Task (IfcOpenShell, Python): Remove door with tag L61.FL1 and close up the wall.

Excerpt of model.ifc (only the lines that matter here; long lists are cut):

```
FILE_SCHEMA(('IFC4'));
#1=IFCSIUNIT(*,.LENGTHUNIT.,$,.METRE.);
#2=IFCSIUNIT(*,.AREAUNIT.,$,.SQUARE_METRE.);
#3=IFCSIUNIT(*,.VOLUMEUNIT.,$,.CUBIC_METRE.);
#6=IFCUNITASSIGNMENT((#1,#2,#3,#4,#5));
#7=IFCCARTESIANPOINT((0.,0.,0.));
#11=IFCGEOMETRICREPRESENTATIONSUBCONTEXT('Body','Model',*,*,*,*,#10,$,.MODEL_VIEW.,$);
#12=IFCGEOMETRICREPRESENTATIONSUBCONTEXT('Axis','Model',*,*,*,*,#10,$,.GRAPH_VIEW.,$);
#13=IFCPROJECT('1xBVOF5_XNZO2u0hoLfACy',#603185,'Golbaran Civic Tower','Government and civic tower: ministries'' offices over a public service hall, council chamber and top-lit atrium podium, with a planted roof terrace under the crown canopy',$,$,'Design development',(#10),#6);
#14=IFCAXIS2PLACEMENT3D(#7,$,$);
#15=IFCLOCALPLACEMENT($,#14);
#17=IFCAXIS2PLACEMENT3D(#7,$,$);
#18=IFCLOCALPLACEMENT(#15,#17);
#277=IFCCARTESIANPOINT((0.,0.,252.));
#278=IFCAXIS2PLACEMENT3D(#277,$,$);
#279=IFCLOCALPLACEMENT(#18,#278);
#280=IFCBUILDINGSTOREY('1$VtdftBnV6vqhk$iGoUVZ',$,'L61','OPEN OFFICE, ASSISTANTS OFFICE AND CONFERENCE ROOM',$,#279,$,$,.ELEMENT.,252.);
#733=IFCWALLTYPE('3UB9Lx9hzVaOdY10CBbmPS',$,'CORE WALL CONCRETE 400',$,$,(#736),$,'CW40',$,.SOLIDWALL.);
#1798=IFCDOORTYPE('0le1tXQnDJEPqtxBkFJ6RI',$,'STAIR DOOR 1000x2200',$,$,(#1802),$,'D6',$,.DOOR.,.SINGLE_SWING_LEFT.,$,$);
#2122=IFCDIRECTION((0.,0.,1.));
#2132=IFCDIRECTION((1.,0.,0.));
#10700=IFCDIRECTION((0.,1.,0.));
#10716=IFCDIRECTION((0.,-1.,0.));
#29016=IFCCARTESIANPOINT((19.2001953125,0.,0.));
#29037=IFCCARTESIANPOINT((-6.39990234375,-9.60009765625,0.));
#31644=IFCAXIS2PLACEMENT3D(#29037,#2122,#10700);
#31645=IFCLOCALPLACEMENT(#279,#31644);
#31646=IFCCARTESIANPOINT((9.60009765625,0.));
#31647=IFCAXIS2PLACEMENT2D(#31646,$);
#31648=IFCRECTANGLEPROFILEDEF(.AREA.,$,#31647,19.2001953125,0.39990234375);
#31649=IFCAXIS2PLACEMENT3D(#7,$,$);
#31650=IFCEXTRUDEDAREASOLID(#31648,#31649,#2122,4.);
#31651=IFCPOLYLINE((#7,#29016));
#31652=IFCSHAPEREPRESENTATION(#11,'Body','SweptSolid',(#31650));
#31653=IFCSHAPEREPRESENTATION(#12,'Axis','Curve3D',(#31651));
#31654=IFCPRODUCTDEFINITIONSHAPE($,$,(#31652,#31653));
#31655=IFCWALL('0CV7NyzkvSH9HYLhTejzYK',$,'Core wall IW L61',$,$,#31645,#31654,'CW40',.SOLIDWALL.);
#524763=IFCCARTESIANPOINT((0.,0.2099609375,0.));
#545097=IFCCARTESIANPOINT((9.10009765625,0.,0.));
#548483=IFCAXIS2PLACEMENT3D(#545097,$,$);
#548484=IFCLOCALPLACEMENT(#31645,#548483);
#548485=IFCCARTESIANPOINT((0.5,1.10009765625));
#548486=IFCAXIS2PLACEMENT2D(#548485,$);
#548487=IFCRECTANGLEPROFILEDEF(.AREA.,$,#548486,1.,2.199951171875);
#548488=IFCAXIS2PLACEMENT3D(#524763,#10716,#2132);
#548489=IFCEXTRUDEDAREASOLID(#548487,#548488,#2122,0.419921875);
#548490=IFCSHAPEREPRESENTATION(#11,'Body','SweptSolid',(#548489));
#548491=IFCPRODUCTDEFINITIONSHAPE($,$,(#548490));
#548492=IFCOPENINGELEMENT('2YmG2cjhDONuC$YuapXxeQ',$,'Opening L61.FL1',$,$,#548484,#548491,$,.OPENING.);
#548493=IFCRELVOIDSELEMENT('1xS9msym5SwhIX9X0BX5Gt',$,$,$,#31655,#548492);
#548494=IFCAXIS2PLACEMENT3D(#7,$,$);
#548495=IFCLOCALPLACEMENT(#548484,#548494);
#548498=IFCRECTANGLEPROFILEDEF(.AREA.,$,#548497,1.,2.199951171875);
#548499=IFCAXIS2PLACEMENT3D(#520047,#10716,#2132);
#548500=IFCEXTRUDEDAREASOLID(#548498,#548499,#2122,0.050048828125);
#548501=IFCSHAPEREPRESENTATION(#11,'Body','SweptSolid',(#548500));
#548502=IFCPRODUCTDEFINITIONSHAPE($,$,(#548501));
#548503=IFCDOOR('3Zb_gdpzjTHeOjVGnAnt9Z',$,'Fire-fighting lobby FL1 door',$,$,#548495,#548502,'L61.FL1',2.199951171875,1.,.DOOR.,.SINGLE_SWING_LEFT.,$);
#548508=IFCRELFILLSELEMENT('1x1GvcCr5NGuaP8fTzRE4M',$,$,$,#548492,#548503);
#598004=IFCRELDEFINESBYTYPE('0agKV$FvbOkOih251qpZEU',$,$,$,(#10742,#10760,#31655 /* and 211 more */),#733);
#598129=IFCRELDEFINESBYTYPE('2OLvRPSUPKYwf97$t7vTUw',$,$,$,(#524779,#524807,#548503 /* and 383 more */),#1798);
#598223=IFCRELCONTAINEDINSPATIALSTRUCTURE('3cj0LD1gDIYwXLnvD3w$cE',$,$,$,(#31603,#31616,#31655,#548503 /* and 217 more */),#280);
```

```python
import ifcopenshell
import ifcopenshell.api.feature
import ifcopenshell.api.root
import ifcopenshell.geom
import ifcopenshell.util.shape

model = ifcopenshell.open("model.ifc")
settings = ifcopenshell.geom.settings()


def volume(element):
    """Net volume in cubic metres, openings subtracted."""
    shape = ifcopenshell.geom.create_shape(settings, element)
    return ifcopenshell.util.shape.get_volume(shape.geometry)


door = model.by_guid("3Zb_gdpzjTHeOjVGnAnt9Z")
opening = door.FillsVoids[0].RelatingOpeningElement
wall = opening.VoidsElements[0].RelatingBuildingElement
before = volume(wall)

ifcopenshell.api.root.remove_product(model, product=door)
ifcopenshell.api.feature.remove_feature(model, feature=opening)

after = volume(wall)

print(f"wall volume {before:.3f} -> {after:.3f} m3")

model.write("model_edited.ifc")
```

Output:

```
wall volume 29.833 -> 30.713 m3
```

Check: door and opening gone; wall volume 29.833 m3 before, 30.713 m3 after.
